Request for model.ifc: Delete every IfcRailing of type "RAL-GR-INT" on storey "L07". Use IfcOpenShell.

First a look at what the model holds.

```python
import ifcopenshell
import ifcopenshell.util.element

model = ifcopenshell.open("model.ifc")
print(model.schema)
storey = next(s for s in model.by_type("IfcBuildingStorey") if s.Name == "L07")
railings = [e for e in ifcopenshell.util.element.get_decomposition(storey) if e.is_a("IfcRailing")]
seen = {}
for e in railings:
    element_type = ifcopenshell.util.element.get_type(e)
    name = element_type.Name if element_type not in (None, e) else None
    seen[name] = seen.get(name, 0) + 1
for name, count in sorted(seen.items(), key=str):
    print(count, "x", name)
```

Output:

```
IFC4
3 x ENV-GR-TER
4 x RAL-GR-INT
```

```python
import ifcopenshell
import ifcopenshell.api.root
import ifcopenshell.util.element

model = ifcopenshell.open("model.ifc")

storey = next(s for s in model.by_type("IfcBuildingStorey") if s.Name == "L07")
railings = [e for e in ifcopenshell.util.element.get_decomposition(storey) if e.is_a("IfcRailing")]
targets = [e for e in railings if (t := ifcopenshell.util.element.get_type(e)) not in (None, e) and t.Name == "RAL-GR-INT"]

for e in targets:
    ifcopenshell.api.root.remove_product(model, product=e)
print(len(targets), "removed")

model.write("model_edited.ifc")
```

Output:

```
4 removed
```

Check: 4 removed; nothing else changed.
